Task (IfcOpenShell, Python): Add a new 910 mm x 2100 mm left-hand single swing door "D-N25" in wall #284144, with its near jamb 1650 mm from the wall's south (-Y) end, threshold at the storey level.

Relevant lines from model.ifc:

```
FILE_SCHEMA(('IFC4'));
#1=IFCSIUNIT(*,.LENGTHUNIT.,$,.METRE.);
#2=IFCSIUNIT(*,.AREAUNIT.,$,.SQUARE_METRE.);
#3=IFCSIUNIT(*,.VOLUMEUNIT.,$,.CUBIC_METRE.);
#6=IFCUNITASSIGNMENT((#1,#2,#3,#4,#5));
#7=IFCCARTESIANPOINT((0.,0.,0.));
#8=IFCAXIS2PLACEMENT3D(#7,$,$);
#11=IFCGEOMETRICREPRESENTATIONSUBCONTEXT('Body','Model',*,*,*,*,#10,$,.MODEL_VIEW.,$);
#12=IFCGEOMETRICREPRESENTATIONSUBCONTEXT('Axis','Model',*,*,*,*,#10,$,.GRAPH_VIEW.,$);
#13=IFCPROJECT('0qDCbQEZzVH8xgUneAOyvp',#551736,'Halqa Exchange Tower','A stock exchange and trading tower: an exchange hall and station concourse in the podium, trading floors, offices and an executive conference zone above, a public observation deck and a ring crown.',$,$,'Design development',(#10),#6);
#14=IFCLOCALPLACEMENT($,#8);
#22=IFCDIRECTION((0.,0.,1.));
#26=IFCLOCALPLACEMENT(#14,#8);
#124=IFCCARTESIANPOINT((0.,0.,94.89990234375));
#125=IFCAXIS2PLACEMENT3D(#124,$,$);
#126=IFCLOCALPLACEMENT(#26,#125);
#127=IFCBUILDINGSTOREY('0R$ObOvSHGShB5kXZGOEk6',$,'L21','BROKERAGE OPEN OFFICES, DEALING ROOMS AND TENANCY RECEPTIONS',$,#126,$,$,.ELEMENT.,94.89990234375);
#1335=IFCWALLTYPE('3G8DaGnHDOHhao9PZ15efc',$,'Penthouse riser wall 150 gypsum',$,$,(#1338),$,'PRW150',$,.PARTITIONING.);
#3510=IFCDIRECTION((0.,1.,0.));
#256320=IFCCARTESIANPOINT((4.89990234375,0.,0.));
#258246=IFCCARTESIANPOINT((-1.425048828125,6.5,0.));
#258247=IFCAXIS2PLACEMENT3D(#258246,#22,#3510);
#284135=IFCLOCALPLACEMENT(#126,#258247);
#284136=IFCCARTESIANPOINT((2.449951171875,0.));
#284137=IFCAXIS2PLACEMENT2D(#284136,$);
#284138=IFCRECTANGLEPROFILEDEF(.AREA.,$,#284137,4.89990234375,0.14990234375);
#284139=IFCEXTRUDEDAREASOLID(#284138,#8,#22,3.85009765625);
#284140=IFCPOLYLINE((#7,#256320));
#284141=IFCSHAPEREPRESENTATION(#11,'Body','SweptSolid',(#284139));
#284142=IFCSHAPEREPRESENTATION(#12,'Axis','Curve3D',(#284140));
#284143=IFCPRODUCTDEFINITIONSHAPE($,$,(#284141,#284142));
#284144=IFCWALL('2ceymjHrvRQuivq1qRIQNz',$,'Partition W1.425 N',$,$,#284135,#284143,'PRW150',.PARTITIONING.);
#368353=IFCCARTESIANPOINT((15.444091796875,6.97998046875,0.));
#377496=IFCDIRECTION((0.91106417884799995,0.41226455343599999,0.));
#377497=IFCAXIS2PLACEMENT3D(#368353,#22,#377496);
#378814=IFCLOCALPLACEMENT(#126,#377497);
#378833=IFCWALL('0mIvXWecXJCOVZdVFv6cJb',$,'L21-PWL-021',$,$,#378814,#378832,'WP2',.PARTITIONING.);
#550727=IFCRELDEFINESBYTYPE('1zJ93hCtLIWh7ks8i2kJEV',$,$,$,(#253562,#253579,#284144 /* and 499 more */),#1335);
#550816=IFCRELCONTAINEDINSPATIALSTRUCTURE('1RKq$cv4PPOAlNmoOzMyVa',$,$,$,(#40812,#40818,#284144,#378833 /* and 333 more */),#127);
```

```python
import numpy as np
import ifcopenshell
import ifcopenshell.api.feature
import ifcopenshell.api.geometry
import ifcopenshell.api.root
import ifcopenshell.api.spatial
import ifcopenshell.geom
import ifcopenshell.util.element
import ifcopenshell.util.placement
import ifcopenshell.util.representation
import ifcopenshell.util.shape
import ifcopenshell.util.unit

model = ifcopenshell.open("model.ifc")
unit_scale = ifcopenshell.util.unit.calculate_unit_scale(model)
settings = ifcopenshell.geom.settings()


def volume(element):
    """Net volume in cubic metres, openings subtracted."""
    shape = ifcopenshell.geom.create_shape(settings, element)
    return ifcopenshell.util.shape.get_volume(shape.geometry)


wall = model.by_guid("2ceymjHrvRQuivq1qRIQNz")
storey = ifcopenshell.util.element.get_container(wall, ifc_class="IfcBuildingStorey")
context = ifcopenshell.util.representation.get_context(model, "Model", "Body", "MODEL_VIEW")
before = volume(wall)

width, height, from_end, sill = 0.91, 2.1, 1.65, 0.0  # metres

# The wall runs along its own X axis, and the end named is its -X end.
wall_shape = ifcopenshell.geom.create_shape(settings, wall)
x, y, z = ifcopenshell.util.shape.get_vertices(wall_shape.geometry).T
start = x.min() + from_end
face, thickness = float(y.min()), float(y.max() - y.min())
wall_matrix = ifcopenshell.util.placement.get_local_placement(wall.ObjectPlacement)
level = ifcopenshell.util.placement.get_local_placement(storey.ObjectPlacement)[2, 3]


def in_wall(x, y):
    """Placement at x, y metres in the wall's axes, at sill height."""
    matrix = wall_matrix.copy()
    matrix[:, 3] = wall_matrix @ np.array([x / unit_scale, y / unit_scale, 0.0, 1.0])
    matrix[2, 3] = level + sill / unit_scale
    return matrix


# Opening: a box that overshoots both wall faces by 50 mm.
opening = ifcopenshell.api.root.create_entity(model, ifc_class="IfcOpeningElement", predefined_type="OPENING")
box = ifcopenshell.api.geometry.add_wall_representation(
    model, context=context, length=width, height=height, thickness=thickness + 0.1
)
ifcopenshell.api.geometry.assign_representation(model, product=opening, representation=box)
ifcopenshell.api.geometry.edit_object_placement(model, product=opening, matrix=in_wall(start, face - 0.05), is_si=False)
ifcopenshell.api.feature.add_feature(model, feature=opening, element=wall)

door = ifcopenshell.api.root.create_entity(model, ifc_class="IfcDoor", name="D-N25", predefined_type="DOOR")
door.OverallWidth, door.OverallHeight = width / unit_scale, height / unit_scale
door.OperationType = "SINGLE_SWING_LEFT"
body = ifcopenshell.api.geometry.add_door_representation(
    model,
    context=context,
    overall_width=door.OverallWidth,
    overall_height=door.OverallHeight,
    operation_type="SINGLE_SWING_LEFT",
    lining_properties={"LiningDepth": thickness / unit_scale, "ThresholdDepth": thickness / unit_scale},
)
ifcopenshell.api.geometry.assign_representation(model, product=door, representation=body)
ifcopenshell.api.spatial.assign_container(model, products=[door], relating_structure=storey)
ifcopenshell.api.feature.add_filling(model, opening=opening, element=door)

# The lining spans the wall, so the door starts at the wall face.
ifcopenshell.api.geometry.edit_object_placement(model, product=door, matrix=in_wall(start, face), is_si=False)

after = volume(wall)

print(f"wall volume {before:.3f} -> {after:.3f} m3")

model.write("model_updated.ifc")
```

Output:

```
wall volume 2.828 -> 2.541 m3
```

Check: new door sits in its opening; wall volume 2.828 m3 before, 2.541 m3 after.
